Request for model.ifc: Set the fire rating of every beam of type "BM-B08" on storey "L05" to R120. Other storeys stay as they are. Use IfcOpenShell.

First a look at what the model holds.

```python
import ifcopenshell
import ifcopenshell.util.element

model = ifcopenshell.open("model.ifc")
print(model.schema)
storey = next(s for s in model.by_type("IfcBuildingStorey") if s.Name == "L05")
beams = [e for e in ifcopenshell.util.element.get_decomposition(storey) if e.is_a("IfcBeam")]
seen = {}
for e in beams:
    element_type = ifcopenshell.util.element.get_type(e)
    key = (element_type.Name if element_type != e and element_type else None, ifcopenshell.util.element.get_pset(e, "Pset_BeamCommon", "FireRating"))
    seen[key] = seen.get(key, 0) + 1
for (name, value), count in sorted(seen.items(), key=str):
    print(count, "x", name, "|", value)
```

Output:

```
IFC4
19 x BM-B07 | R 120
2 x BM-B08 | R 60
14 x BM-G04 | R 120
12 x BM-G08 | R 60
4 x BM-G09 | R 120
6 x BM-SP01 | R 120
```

```python
import ifcopenshell
import ifcopenshell.api.pset
import ifcopenshell.util.element

model = ifcopenshell.open("model.ifc")

storey = next(s for s in model.by_type("IfcBuildingStorey") if s.Name == "L05")
beams = [e for e in ifcopenshell.util.element.get_decomposition(storey) if e.is_a("IfcBeam")]

count = 0
for e in beams:
    element_type = ifcopenshell.util.element.get_type(e)
    if element_type in (None, e) or element_type.Name != "BM-B08":
        continue
    # add_pset returns the element's existing set when there is one.
    pset = ifcopenshell.api.pset.add_pset(model, product=e, name="Pset_BeamCommon")
    ifcopenshell.api.pset.edit_pset(model, pset=pset, properties={"FireRating": "R120"})
    count += 1

print(count, "beams updated")

model.write("model_edited.ifc")
```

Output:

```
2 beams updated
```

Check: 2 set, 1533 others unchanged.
